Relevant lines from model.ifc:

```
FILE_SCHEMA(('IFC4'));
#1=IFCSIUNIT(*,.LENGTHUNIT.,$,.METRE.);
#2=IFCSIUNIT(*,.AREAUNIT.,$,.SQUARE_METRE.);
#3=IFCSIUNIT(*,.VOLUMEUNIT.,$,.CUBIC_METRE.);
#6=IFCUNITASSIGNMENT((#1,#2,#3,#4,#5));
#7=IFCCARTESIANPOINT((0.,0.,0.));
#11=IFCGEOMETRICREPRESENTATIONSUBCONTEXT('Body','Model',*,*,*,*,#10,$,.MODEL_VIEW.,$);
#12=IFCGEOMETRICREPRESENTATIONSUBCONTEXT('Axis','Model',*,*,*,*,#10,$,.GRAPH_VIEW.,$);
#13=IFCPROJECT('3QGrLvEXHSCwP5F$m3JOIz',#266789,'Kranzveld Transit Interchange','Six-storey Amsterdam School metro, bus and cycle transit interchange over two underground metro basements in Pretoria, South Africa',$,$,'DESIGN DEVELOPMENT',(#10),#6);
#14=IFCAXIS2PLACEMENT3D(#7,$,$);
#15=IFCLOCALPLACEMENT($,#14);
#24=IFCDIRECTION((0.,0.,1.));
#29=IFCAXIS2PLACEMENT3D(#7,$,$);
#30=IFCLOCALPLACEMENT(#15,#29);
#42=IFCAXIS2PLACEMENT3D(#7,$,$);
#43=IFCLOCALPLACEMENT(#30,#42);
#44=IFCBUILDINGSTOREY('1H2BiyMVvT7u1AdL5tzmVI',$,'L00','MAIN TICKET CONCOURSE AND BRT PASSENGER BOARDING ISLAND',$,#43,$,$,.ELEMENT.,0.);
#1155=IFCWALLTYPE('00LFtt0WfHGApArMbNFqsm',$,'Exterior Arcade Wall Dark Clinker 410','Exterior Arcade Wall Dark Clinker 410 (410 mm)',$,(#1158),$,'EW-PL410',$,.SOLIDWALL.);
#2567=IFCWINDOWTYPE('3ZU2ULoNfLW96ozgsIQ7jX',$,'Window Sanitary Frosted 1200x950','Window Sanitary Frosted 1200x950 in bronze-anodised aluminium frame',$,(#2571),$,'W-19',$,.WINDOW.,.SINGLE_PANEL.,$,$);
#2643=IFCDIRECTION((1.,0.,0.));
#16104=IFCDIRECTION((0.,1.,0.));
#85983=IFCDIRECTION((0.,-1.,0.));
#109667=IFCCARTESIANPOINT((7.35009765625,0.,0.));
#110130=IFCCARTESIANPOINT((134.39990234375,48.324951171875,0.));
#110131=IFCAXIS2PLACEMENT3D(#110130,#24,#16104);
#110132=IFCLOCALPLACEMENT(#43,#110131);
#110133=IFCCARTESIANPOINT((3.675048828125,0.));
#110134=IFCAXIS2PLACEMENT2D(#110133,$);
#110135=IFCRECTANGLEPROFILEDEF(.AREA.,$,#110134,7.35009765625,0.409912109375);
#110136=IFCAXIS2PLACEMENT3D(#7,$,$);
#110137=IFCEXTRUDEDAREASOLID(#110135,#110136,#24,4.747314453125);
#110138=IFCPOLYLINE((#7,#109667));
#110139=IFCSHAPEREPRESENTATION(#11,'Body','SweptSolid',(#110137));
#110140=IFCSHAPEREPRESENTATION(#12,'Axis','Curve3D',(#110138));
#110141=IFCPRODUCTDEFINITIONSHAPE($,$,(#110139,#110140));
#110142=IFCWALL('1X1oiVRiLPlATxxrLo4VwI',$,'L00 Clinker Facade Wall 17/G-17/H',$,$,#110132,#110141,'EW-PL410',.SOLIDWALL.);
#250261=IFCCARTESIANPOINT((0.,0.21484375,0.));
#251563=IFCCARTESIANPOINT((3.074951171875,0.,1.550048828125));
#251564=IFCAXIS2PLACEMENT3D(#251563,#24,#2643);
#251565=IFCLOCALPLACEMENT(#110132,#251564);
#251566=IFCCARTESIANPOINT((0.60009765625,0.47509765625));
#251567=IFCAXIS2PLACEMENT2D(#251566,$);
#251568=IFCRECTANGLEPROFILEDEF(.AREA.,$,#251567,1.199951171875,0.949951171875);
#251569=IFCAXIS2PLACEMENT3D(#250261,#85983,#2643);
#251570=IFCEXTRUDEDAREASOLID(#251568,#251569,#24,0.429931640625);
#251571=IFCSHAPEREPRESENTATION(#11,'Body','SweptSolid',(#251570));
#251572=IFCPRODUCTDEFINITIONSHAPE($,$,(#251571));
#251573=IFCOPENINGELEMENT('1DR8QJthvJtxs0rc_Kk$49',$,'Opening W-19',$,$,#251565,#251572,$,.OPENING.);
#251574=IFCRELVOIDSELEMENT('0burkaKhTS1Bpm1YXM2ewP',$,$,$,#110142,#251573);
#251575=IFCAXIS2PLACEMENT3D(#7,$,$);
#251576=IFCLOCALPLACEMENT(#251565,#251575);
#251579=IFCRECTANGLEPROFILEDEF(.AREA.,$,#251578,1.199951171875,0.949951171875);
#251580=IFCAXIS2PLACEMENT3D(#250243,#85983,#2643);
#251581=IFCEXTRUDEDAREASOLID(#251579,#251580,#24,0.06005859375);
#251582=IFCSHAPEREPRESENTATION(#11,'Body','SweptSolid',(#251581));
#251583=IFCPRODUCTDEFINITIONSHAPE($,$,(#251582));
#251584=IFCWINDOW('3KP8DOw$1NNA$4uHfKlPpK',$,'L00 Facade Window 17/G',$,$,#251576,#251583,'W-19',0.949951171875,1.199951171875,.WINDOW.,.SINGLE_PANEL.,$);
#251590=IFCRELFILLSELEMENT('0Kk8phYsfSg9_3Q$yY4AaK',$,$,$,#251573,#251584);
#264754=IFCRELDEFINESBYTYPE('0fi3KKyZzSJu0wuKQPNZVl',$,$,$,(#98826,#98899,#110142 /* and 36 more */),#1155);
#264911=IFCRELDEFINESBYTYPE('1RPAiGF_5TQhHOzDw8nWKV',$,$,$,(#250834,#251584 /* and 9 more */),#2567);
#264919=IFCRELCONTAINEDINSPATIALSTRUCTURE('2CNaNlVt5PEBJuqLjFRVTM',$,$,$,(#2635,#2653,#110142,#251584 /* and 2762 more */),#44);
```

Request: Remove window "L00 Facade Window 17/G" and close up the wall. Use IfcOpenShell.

```python
import ifcopenshell
import ifcopenshell.api.feature
import ifcopenshell.api.root
import ifcopenshell.geom
import ifcopenshell.util.shape

model = ifcopenshell.open("model.ifc")
settings = ifcopenshell.geom.settings()


def volume(element):
    """Net volume in cubic metres, openings subtracted."""
    shape = ifcopenshell.geom.create_shape(settings, element)
    return ifcopenshell.util.shape.get_volume(shape.geometry)


window = model.by_guid("3KP8DOw$1NNA$4uHfKlPpK")
opening = window.FillsVoids[0].RelatingOpeningElement
wall = opening.VoidsElements[0].RelatingBuildingElement
before = volume(wall)

ifcopenshell.api.root.remove_product(model, product=window)
ifcopenshell.api.feature.remove_feature(model, feature=opening)

after = volume(wall)

print(f"wall volume {before:.3f} -> {after:.3f} m3")

model.write("model_edited.ifc")
```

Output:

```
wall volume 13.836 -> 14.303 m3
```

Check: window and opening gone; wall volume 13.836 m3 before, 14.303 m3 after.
